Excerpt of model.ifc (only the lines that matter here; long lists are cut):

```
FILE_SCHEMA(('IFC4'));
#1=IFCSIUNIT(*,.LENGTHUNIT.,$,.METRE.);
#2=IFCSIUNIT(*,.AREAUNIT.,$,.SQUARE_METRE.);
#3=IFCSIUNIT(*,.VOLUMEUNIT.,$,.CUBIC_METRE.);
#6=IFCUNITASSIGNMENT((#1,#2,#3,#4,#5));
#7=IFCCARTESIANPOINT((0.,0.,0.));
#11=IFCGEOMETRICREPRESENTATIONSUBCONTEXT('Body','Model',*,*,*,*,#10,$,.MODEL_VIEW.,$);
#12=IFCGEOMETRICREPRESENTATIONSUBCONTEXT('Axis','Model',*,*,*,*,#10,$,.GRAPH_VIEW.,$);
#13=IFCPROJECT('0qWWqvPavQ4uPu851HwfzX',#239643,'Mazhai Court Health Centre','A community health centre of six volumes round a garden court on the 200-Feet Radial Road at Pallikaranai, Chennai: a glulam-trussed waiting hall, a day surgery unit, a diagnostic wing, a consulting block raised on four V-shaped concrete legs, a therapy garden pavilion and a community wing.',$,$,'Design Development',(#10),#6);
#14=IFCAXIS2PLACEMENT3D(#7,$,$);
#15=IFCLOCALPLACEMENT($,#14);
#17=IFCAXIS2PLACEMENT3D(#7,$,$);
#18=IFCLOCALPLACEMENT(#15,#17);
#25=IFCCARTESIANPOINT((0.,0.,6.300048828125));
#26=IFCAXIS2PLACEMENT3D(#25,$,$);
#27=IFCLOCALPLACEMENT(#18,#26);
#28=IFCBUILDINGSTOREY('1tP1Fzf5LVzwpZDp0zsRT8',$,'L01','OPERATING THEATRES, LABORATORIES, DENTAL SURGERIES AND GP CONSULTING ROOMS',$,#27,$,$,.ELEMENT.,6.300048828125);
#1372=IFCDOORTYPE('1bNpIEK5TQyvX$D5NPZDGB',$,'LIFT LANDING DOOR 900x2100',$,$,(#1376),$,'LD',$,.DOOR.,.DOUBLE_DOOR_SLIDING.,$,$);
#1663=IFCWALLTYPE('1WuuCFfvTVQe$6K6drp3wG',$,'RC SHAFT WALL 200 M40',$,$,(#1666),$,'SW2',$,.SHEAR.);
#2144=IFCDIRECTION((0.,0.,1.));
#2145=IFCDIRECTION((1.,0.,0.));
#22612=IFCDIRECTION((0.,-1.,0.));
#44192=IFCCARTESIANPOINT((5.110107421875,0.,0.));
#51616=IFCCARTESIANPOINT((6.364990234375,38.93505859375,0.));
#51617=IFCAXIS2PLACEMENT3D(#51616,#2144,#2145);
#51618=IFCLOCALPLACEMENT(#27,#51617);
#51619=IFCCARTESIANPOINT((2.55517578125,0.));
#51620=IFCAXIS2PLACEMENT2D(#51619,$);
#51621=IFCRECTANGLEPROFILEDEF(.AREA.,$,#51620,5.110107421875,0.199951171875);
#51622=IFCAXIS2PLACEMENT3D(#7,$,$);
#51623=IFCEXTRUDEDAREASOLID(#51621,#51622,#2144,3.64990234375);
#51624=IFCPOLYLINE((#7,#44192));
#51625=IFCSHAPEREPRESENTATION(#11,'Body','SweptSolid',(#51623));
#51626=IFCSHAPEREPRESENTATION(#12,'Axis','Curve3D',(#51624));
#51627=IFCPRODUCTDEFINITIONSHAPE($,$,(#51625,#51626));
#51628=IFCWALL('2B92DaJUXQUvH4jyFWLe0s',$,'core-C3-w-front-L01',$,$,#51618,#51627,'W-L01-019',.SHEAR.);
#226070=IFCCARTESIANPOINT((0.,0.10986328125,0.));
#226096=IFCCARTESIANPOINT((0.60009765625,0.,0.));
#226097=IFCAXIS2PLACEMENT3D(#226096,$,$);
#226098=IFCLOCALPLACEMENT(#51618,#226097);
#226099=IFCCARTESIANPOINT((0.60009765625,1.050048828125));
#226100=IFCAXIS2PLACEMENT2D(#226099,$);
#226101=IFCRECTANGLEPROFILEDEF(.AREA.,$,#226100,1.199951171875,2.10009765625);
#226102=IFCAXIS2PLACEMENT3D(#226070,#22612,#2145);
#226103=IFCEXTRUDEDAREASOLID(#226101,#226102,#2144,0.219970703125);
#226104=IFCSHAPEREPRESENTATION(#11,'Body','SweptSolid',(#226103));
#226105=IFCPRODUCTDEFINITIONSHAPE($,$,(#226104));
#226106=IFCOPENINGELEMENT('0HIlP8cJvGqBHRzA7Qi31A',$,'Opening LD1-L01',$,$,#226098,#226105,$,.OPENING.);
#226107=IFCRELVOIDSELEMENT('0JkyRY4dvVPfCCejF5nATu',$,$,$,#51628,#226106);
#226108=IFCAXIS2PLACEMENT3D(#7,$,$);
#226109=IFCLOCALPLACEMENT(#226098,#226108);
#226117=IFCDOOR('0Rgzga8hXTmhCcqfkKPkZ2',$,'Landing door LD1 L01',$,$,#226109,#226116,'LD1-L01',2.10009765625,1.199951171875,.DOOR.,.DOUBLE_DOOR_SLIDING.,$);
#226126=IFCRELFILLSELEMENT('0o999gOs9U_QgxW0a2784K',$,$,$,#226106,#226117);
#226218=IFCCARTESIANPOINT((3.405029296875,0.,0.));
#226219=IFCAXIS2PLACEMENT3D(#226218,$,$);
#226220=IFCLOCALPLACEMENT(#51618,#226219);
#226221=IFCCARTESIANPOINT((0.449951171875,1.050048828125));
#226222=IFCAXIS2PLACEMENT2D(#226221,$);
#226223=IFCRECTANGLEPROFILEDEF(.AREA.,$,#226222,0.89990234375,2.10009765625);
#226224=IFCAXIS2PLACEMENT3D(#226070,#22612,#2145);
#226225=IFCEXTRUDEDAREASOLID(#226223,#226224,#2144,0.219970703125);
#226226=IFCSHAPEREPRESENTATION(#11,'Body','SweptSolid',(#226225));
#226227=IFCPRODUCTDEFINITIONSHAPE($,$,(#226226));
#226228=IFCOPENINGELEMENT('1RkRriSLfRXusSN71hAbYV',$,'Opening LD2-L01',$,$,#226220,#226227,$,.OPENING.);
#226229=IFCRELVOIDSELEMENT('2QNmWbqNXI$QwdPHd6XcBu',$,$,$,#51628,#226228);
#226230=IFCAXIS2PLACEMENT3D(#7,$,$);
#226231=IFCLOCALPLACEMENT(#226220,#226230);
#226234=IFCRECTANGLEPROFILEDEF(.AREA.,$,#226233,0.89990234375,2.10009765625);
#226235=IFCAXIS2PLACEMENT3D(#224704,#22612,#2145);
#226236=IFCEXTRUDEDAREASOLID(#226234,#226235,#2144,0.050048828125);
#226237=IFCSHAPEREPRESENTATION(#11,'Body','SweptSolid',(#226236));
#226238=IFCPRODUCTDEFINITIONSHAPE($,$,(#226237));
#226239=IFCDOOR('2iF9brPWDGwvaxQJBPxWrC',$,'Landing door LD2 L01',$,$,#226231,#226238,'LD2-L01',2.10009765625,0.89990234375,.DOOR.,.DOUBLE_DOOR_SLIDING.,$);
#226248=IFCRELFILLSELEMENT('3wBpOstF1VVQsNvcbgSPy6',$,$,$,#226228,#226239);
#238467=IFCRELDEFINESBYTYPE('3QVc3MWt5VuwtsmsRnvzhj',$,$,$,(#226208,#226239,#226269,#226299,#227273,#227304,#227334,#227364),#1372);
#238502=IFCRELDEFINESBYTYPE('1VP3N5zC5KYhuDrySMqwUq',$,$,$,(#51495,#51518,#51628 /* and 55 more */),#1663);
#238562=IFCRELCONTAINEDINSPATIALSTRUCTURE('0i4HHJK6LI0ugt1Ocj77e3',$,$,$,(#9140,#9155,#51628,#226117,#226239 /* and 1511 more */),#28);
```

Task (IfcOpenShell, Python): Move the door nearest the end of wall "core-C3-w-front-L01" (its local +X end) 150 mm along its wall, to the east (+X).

```python
import ifcopenshell
import ifcopenshell.api.geometry
import ifcopenshell.util.placement
import ifcopenshell.util.unit

model = ifcopenshell.open("model.ifc")
unit_scale = ifcopenshell.util.unit.calculate_unit_scale(model)

door = model.by_guid("2iF9brPWDGwvaxQJBPxWrC")
opening = door.FillsVoids[0].RelatingOpeningElement
wall = opening.VoidsElements[0].RelatingBuildingElement

wall_matrix = ifcopenshell.util.placement.get_local_placement(wall.ObjectPlacement)
shift = wall_matrix[:3, 0] * 0.15 / unit_scale
before = ifcopenshell.util.placement.get_local_placement(door.ObjectPlacement)[:3, 3].copy()

# The door is placed relative to its opening, so it follows when the opening moves.
matrix = ifcopenshell.util.placement.get_local_placement(opening.ObjectPlacement)
matrix[:3, 3] += shift
ifcopenshell.api.geometry.edit_object_placement(
    model, product=opening, matrix=matrix, is_si=False, should_transform_children=True
)

after = ifcopenshell.util.placement.get_local_placement(door.ObjectPlacement)[:3, 3]
print("door moved by", (after - before).round(3) + 0.0)

model.write("model_updated.ifc")
```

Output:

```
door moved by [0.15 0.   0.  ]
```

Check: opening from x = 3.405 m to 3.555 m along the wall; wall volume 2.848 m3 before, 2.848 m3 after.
